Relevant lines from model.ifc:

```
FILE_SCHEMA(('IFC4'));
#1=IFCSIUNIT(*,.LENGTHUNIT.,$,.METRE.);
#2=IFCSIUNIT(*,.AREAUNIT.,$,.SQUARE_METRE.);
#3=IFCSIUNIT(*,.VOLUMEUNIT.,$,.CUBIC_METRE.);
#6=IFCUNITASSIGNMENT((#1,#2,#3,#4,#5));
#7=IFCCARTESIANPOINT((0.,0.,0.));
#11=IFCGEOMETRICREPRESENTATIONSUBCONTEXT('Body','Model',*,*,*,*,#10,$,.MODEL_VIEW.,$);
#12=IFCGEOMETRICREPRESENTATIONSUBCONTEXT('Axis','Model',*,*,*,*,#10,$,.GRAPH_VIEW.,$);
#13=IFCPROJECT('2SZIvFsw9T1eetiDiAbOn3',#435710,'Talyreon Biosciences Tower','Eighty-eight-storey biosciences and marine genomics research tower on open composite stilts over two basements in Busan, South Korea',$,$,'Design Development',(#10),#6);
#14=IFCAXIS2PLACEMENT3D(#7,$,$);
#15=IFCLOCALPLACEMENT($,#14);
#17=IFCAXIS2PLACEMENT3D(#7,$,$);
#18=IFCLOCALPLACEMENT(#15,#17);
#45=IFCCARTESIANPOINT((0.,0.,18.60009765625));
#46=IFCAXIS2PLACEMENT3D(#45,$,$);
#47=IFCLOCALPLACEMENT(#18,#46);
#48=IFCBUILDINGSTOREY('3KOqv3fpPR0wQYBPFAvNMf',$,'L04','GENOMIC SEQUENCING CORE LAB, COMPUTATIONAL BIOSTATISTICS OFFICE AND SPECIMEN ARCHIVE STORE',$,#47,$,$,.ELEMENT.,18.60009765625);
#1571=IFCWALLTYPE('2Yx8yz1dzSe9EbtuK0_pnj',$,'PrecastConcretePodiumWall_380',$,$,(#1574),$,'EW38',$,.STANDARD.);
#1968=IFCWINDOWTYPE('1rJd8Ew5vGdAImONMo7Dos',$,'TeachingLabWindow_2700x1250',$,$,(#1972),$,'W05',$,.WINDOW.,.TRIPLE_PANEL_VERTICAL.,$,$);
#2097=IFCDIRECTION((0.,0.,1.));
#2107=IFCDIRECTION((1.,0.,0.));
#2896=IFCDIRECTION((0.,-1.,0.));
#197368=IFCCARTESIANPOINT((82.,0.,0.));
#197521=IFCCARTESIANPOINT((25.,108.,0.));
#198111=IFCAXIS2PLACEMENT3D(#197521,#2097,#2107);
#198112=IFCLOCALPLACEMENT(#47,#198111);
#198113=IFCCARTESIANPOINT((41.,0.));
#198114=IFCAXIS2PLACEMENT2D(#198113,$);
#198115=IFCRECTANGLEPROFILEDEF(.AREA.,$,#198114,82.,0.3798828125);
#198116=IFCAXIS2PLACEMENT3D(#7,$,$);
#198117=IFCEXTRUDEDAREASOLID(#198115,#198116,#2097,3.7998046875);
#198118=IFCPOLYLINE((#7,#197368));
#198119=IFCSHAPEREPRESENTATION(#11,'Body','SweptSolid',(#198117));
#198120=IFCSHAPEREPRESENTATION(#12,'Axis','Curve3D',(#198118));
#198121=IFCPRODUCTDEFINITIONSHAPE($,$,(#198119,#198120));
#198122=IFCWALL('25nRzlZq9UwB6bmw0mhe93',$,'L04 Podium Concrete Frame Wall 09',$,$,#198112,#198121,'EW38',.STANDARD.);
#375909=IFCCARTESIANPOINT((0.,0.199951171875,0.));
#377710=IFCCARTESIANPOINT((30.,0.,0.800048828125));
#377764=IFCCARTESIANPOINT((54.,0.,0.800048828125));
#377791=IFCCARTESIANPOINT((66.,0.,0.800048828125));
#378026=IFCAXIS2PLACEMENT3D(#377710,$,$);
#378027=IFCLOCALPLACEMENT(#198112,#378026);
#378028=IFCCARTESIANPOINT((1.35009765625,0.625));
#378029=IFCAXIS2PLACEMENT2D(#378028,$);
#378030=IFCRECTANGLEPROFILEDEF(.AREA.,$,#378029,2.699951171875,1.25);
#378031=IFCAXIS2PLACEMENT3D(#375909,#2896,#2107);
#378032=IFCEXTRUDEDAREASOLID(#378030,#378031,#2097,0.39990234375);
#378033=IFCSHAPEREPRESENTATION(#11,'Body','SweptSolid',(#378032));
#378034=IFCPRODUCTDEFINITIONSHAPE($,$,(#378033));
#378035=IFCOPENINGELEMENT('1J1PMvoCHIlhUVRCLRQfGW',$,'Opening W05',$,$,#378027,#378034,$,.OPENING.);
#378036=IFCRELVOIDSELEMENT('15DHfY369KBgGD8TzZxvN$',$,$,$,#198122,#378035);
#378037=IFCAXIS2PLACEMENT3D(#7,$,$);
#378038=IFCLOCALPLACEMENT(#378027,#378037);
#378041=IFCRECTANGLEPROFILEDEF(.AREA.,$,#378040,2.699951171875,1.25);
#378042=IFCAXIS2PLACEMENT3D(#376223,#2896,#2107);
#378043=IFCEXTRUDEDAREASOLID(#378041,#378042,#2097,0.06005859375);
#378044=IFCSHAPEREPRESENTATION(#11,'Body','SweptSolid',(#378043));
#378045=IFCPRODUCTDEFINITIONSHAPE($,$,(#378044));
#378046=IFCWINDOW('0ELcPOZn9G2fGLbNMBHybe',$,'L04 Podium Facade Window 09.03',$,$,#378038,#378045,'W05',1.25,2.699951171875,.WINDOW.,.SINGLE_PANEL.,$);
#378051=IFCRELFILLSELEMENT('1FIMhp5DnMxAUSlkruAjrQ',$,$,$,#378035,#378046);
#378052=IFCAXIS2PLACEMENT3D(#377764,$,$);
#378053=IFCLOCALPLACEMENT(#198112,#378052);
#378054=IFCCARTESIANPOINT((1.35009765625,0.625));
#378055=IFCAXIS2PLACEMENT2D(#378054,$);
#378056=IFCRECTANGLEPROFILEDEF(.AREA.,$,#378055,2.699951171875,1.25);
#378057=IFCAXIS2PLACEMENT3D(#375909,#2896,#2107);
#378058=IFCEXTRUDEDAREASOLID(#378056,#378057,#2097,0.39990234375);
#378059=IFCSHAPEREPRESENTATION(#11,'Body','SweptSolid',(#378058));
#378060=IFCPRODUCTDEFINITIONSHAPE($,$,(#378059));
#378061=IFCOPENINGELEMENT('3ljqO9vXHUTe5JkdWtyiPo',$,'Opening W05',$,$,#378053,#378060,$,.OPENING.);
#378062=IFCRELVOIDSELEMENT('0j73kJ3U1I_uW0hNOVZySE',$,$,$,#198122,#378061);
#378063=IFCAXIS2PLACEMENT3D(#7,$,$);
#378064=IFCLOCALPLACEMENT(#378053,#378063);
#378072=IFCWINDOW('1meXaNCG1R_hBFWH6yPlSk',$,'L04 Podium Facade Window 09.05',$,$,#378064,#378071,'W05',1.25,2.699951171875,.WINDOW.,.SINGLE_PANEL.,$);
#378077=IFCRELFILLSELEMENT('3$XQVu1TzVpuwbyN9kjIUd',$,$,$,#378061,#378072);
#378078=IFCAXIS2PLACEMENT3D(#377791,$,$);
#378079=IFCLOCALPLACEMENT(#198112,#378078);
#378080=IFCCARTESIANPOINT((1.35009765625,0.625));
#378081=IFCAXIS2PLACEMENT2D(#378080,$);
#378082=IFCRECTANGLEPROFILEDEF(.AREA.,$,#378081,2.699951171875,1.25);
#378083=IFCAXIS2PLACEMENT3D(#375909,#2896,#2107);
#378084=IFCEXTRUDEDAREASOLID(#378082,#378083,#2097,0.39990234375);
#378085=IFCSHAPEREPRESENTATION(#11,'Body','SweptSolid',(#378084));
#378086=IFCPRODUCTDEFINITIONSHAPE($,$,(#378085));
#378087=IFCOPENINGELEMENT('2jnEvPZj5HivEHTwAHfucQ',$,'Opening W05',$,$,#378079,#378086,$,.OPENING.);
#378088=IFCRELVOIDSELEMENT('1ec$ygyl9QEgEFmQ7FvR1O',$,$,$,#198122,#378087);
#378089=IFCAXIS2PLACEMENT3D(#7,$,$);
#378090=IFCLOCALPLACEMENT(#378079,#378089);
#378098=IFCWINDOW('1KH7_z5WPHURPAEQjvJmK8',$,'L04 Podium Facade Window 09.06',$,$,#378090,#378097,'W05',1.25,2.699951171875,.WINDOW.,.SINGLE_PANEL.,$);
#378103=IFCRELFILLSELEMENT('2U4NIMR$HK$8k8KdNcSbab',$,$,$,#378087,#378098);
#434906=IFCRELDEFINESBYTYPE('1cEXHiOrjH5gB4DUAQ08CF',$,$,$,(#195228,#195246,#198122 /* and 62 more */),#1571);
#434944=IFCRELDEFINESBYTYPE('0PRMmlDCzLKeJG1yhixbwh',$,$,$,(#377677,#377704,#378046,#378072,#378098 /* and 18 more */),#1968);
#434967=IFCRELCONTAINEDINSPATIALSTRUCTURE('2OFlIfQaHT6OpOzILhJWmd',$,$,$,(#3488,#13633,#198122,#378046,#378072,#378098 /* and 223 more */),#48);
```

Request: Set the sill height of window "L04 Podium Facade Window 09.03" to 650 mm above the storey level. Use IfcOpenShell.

```python
import numpy as np
import ifcopenshell
import ifcopenshell.api.geometry
import ifcopenshell.geom
import ifcopenshell.util.element
import ifcopenshell.util.placement
import ifcopenshell.util.shape
import ifcopenshell.util.unit

model = ifcopenshell.open("model.ifc")
unit_scale = ifcopenshell.util.unit.calculate_unit_scale(model)

window = model.by_guid("0ELcPOZn9G2fGLbNMBHybe")
opening = window.FillsVoids[0].RelatingOpeningElement
storey = ifcopenshell.util.element.get_container(window, ifc_class="IfcBuildingStorey")
level = ifcopenshell.util.placement.get_local_placement(storey.ObjectPlacement)[2, 3]

# The opening's origin need not be at the sill, so measure its lowest point.
shape = ifcopenshell.geom.create_shape(ifcopenshell.geom.settings(), opening)
bottom = ifcopenshell.util.shape.get_shape_bottom_elevation(shape, shape.geometry) / unit_scale
dz = level + 0.65 / unit_scale - bottom

shift = np.array([0.0, 0.0, dz])
# The window is placed relative to its opening, so it follows when the opening moves.
matrix = ifcopenshell.util.placement.get_local_placement(opening.ObjectPlacement)
matrix[:3, 3] += shift
ifcopenshell.api.geometry.edit_object_placement(
    model, product=opening, matrix=matrix, is_si=False, should_transform_children=True
)

print(f"moved by {dz * unit_scale:+.3f} m")

model.write("model_updated.ifc")
```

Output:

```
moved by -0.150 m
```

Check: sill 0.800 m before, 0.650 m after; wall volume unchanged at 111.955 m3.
